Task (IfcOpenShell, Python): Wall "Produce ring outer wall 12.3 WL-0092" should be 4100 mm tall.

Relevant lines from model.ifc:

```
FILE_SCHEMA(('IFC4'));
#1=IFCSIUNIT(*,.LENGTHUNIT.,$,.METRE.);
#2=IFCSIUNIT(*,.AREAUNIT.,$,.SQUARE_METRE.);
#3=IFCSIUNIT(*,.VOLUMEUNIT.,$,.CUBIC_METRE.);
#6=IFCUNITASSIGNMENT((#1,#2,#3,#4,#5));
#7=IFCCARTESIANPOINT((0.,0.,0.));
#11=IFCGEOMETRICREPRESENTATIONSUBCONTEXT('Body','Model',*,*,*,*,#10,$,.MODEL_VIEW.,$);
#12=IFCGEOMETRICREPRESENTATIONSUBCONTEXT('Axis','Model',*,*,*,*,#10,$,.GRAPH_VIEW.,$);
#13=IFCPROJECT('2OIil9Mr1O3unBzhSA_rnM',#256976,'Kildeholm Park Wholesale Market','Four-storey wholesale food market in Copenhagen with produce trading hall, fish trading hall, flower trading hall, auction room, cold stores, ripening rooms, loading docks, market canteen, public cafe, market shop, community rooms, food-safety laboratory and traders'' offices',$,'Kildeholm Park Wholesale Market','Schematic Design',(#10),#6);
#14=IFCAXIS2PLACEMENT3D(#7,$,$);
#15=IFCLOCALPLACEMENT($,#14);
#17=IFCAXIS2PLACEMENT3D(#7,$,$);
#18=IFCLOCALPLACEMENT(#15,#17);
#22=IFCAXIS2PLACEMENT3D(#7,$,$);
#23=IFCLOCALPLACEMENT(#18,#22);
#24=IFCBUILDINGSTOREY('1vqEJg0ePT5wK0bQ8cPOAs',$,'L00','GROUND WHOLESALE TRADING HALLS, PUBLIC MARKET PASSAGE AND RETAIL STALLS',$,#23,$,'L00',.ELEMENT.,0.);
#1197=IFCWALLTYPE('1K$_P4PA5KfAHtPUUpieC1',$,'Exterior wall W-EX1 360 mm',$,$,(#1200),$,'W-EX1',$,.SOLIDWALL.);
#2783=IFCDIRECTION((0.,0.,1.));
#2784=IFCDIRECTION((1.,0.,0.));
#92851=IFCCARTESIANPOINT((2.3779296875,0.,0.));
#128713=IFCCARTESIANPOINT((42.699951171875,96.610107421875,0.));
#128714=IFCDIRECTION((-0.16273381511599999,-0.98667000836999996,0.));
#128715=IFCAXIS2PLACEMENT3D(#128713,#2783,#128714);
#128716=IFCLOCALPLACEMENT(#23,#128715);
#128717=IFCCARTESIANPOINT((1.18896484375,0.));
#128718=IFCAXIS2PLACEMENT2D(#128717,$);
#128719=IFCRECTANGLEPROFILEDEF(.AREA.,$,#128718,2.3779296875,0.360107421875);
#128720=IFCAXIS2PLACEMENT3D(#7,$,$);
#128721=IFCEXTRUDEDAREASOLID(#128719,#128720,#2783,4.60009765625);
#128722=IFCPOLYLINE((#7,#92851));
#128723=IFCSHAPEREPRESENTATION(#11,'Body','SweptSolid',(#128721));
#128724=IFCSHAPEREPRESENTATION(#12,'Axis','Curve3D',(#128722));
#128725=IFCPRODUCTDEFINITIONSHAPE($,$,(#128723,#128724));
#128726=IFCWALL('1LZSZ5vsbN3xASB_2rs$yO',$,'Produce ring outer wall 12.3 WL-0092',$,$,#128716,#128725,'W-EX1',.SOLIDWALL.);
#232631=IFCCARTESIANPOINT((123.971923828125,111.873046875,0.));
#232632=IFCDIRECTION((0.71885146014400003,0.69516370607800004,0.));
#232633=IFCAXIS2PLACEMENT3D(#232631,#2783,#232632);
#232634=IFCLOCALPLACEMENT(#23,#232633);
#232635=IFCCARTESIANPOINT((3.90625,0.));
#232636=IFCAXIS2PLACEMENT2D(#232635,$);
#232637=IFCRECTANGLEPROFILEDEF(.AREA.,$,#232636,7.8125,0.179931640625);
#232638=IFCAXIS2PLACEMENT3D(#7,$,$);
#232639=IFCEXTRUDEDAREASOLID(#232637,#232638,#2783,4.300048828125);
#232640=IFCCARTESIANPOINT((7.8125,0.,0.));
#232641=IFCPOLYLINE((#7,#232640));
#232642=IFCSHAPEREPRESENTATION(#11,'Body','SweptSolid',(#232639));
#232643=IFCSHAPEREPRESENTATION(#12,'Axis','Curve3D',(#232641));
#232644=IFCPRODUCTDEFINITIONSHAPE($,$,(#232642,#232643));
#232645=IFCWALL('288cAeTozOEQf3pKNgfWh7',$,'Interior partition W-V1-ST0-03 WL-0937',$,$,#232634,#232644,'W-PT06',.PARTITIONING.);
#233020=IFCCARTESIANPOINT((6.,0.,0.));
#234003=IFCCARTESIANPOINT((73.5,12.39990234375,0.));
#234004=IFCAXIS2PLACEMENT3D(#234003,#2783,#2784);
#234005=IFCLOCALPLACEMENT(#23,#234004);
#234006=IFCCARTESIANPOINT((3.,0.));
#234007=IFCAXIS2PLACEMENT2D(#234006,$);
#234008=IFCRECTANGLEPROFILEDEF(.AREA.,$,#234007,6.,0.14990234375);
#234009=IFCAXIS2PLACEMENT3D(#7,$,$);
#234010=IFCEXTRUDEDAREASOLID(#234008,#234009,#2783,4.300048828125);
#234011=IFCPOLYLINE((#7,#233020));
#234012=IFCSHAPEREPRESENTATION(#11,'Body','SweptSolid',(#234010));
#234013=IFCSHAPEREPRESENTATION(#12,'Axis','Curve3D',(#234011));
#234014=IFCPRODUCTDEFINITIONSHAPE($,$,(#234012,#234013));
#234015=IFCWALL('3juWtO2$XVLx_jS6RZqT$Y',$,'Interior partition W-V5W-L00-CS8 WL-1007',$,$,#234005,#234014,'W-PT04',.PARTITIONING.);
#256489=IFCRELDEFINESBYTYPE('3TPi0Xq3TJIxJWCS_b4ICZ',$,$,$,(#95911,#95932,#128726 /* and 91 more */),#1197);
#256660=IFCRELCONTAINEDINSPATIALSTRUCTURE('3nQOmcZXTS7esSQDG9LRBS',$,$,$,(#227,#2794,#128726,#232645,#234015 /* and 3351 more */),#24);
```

```python
import ifcopenshell
import ifcopenshell.geom
import ifcopenshell.util.representation
import ifcopenshell.util.shape
import ifcopenshell.util.unit

model = ifcopenshell.open("model.ifc")
unit_scale = ifcopenshell.util.unit.calculate_unit_scale(model)
settings = ifcopenshell.geom.settings()


def volume(element):
    """Net volume in cubic metres, openings subtracted."""
    shape = ifcopenshell.geom.create_shape(settings, element)
    return ifcopenshell.util.shape.get_volume(shape.geometry)


wall = model.by_guid("1LZSZ5vsbN3xASB_2rs$yO")
before = volume(wall)

body = ifcopenshell.util.representation.get_representation(wall, "Model", "Body")
solid = body.Items[0]
old_height = solid.Depth
solid.Depth = 4.1 / unit_scale
after = volume(wall)

print(f"height {old_height:g} -> {solid.Depth:g}, volume {before:.3f} -> {after:.3f} m3")

model.write("model_rev.ifc")
```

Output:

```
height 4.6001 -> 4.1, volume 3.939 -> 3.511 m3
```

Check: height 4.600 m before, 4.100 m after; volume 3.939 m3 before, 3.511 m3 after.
